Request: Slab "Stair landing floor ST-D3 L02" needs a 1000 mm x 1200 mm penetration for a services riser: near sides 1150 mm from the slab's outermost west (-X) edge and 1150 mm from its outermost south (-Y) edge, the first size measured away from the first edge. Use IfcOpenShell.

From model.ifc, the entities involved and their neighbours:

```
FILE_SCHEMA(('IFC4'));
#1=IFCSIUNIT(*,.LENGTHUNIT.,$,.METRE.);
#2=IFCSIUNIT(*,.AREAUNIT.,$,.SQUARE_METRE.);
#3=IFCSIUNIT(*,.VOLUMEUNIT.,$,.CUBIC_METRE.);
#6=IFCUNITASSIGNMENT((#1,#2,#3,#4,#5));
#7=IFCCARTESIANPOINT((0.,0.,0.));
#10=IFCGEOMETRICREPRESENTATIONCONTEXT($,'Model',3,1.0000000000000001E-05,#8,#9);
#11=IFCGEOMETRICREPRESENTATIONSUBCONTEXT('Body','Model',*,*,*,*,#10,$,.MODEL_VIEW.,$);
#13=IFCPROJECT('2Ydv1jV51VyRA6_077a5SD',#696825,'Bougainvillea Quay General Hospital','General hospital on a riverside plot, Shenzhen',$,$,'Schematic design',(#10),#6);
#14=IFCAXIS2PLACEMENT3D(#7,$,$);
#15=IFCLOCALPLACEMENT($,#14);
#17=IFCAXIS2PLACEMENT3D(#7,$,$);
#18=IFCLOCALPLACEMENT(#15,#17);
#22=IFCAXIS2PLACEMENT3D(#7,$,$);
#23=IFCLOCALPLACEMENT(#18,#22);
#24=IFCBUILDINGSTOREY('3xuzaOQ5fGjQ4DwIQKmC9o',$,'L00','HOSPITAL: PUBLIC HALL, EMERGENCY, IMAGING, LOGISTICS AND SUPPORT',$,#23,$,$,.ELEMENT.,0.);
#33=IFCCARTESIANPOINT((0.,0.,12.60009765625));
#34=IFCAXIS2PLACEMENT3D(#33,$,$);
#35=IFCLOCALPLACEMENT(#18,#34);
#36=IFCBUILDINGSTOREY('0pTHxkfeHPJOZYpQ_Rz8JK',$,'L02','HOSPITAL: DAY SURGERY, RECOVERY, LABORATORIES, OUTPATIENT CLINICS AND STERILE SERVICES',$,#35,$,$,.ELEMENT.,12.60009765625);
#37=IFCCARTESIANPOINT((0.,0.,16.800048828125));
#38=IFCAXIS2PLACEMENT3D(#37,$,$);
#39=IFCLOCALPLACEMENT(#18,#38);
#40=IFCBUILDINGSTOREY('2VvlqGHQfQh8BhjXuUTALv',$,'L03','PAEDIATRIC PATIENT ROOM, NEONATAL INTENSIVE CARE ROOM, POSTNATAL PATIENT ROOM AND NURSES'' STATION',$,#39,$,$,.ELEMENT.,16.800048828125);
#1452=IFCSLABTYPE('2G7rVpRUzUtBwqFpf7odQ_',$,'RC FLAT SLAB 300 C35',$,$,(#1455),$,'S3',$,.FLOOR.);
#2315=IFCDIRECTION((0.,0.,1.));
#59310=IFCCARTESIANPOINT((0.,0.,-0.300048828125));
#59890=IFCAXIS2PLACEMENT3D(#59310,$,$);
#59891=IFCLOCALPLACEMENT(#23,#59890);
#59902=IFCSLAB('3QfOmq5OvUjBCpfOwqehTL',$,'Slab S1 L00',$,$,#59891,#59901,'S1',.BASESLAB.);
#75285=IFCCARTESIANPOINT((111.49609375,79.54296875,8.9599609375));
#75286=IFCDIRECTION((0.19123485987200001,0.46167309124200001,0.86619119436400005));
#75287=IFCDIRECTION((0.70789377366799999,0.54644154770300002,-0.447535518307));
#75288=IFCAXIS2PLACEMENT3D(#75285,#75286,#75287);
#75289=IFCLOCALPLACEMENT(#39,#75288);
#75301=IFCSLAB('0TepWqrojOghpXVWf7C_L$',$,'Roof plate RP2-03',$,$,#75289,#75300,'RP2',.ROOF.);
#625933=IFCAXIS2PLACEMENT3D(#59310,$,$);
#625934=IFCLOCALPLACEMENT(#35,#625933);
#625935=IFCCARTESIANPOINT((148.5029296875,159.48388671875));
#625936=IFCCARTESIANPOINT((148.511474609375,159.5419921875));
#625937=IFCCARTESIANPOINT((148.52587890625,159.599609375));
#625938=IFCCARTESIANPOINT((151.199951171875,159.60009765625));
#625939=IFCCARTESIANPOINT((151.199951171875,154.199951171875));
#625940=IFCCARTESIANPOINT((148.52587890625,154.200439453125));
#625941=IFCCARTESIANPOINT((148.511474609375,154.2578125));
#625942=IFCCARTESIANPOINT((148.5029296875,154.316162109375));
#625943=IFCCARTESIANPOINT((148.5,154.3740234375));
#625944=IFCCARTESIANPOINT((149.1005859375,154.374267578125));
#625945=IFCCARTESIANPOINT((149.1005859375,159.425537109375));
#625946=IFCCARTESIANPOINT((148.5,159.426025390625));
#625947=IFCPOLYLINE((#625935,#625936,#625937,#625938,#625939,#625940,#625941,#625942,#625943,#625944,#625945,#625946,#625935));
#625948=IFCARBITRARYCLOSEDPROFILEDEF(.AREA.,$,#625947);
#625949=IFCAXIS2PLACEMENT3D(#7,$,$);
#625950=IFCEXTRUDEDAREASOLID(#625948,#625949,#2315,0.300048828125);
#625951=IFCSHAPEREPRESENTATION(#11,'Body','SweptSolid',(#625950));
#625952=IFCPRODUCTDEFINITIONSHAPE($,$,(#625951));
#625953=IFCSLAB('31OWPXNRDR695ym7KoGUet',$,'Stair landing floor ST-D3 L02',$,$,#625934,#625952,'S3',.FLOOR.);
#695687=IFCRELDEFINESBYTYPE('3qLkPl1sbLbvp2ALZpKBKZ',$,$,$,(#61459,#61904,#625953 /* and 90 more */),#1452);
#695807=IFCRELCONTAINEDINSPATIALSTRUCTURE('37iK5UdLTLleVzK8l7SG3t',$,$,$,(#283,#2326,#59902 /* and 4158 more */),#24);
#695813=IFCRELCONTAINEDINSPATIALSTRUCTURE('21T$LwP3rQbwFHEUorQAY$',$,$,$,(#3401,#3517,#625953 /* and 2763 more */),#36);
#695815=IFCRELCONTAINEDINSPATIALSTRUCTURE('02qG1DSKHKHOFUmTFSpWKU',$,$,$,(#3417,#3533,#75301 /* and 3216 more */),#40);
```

```python
import numpy as np
import ifcopenshell
import ifcopenshell.api.feature
import ifcopenshell.api.geometry
import ifcopenshell.api.root
import ifcopenshell.geom
import ifcopenshell.util.placement
import ifcopenshell.util.representation
import ifcopenshell.util.shape
import ifcopenshell.util.unit

model = ifcopenshell.open("model.ifc")
unit_scale = ifcopenshell.util.unit.calculate_unit_scale(model)
settings = ifcopenshell.geom.settings()


def volume(element):
    """Net volume in cubic metres, openings subtracted."""
    shape = ifcopenshell.geom.create_shape(settings, element)
    return ifcopenshell.util.shape.get_volume(shape.geometry)


slab = model.by_guid("31OWPXNRDR695ym7KoGUet")
before = volume(slab)

# Extent in the slab's own axes, in metres. The edges named are its -X and -Y sides.
slab_shape = ifcopenshell.geom.create_shape(settings, slab)
vertices = ifcopenshell.util.shape.get_vertices(slab_shape.geometry)
x_min, y_min, bottom = vertices.min(axis=0)
top = vertices[:, 2].max()

opening = ifcopenshell.api.root.create_entity(model, ifc_class="IfcOpeningElement", name="Services riser opening", predefined_type="OPENING")
context = ifcopenshell.util.representation.get_context(model, "Model", "Body", "MODEL_VIEW")
width, depth = 1, 1.2
outline = [(0.0, 0.0), (width, 0.0), (width, depth), (0.0, depth), (0.0, 0.0)]
# Overshoot both faces by 50 mm so the cut is clean.
shape = ifcopenshell.api.geometry.add_slab_representation(
    model, context=context, depth=top - bottom + 0.1, polyline=outline
)
ifcopenshell.api.geometry.assign_representation(model, product=opening, representation=shape)

matrix = ifcopenshell.util.placement.get_local_placement(slab.ObjectPlacement)
matrix[:, 3] = matrix @ np.append(np.array([x_min + 1.15, y_min + 1.15, bottom - 0.05]) / unit_scale, 1.0)
ifcopenshell.api.geometry.edit_object_placement(model, product=opening, matrix=matrix, is_si=False)
ifcopenshell.api.feature.add_feature(model, feature=opening, element=slab)

after = volume(slab)

print(f"slab volume {before:.3f} -> {after:.3f} m3")

model.write("model_edited.ifc")
```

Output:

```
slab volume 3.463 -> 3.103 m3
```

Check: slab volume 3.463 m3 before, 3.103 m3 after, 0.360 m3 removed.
